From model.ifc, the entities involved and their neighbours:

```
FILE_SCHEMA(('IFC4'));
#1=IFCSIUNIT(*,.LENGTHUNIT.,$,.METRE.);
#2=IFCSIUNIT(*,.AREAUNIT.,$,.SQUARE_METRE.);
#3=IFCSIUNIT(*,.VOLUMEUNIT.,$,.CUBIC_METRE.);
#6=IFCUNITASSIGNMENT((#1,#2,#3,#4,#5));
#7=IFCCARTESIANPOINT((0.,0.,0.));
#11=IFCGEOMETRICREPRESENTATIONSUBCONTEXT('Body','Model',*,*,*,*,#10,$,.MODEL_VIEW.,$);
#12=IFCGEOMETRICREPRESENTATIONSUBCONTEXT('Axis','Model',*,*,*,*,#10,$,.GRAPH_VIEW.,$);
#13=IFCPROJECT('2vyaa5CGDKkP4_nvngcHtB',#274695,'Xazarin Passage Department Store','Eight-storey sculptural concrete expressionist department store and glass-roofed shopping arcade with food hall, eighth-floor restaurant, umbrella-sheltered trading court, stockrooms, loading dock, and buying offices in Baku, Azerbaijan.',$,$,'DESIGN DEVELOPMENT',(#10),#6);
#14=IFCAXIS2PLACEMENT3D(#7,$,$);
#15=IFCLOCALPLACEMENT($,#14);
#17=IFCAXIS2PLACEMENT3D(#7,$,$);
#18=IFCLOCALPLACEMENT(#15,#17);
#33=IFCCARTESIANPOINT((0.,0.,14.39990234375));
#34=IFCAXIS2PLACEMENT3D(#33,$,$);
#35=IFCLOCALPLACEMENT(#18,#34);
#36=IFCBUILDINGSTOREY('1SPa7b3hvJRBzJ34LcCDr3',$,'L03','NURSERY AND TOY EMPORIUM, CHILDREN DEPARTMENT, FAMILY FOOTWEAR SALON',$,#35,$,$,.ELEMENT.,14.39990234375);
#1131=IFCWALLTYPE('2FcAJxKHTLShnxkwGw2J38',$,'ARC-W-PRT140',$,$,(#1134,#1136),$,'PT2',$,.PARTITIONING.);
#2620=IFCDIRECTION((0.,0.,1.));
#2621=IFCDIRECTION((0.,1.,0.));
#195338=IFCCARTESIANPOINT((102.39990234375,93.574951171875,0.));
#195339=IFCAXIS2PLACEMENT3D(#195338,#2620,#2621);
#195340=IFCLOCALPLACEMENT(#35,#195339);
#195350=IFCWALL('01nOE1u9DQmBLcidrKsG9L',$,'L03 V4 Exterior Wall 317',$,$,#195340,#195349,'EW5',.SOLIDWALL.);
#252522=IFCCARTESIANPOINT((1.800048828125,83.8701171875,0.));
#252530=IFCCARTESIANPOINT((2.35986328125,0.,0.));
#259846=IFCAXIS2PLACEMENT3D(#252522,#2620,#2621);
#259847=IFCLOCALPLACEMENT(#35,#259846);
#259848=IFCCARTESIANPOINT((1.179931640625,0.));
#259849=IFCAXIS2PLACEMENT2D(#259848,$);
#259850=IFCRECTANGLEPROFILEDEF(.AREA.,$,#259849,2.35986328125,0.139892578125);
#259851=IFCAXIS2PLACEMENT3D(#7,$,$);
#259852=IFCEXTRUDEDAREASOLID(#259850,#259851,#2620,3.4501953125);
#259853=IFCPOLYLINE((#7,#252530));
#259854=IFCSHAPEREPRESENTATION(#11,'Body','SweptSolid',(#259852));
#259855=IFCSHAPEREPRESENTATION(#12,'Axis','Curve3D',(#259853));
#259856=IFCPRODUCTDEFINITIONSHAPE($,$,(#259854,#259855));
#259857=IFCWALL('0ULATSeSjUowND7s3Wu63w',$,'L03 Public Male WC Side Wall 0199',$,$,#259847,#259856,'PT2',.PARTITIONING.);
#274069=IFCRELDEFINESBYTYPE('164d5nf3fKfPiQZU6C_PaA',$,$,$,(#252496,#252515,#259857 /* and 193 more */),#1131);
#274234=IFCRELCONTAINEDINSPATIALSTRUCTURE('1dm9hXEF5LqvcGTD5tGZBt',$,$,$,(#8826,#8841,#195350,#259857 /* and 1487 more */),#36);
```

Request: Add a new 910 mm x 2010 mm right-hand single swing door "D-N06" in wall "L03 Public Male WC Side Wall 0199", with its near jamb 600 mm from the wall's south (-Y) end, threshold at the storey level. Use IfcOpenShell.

```python
import numpy as np
import ifcopenshell
import ifcopenshell.api.feature
import ifcopenshell.api.geometry
import ifcopenshell.api.root
import ifcopenshell.api.spatial
import ifcopenshell.geom
import ifcopenshell.util.element
import ifcopenshell.util.placement
import ifcopenshell.util.representation
import ifcopenshell.util.shape
import ifcopenshell.util.unit

model = ifcopenshell.open("model.ifc")
unit_scale = ifcopenshell.util.unit.calculate_unit_scale(model)
settings = ifcopenshell.geom.settings()


def volume(element):
    """Net volume in cubic metres, openings subtracted."""
    shape = ifcopenshell.geom.create_shape(settings, element)
    return ifcopenshell.util.shape.get_volume(shape.geometry)


wall = model.by_guid("0ULATSeSjUowND7s3Wu63w")
storey = ifcopenshell.util.element.get_container(wall, ifc_class="IfcBuildingStorey")
context = ifcopenshell.util.representation.get_context(model, "Model", "Body", "MODEL_VIEW")
before = volume(wall)

width, height, from_end, sill = 0.91, 2.01, 0.6, 0.0  # metres

# The wall runs along its own X axis, and the end named is its -X end.
wall_shape = ifcopenshell.geom.create_shape(settings, wall)
x, y, z = ifcopenshell.util.shape.get_vertices(wall_shape.geometry).T
start = x.min() + from_end
face, thickness = float(y.min()), float(y.max() - y.min())
wall_matrix = ifcopenshell.util.placement.get_local_placement(wall.ObjectPlacement)
level = ifcopenshell.util.placement.get_local_placement(storey.ObjectPlacement)[2, 3]


def in_wall(x, y):
    """Placement at x, y metres in the wall's axes, at sill height."""
    matrix = wall_matrix.copy()
    matrix[:, 3] = wall_matrix @ np.array([x / unit_scale, y / unit_scale, 0.0, 1.0])
    matrix[2, 3] = level + sill / unit_scale
    return matrix


# Opening: a box that overshoots both wall faces by 50 mm.
opening = ifcopenshell.api.root.create_entity(model, ifc_class="IfcOpeningElement", predefined_type="OPENING")
box = ifcopenshell.api.geometry.add_wall_representation(
    model, context=context, length=width, height=height, thickness=thickness + 0.1
)
ifcopenshell.api.geometry.assign_representation(model, product=opening, representation=box)
ifcopenshell.api.geometry.edit_object_placement(model, product=opening, matrix=in_wall(start, face - 0.05), is_si=False)
ifcopenshell.api.feature.add_feature(model, feature=opening, element=wall)

door = ifcopenshell.api.root.create_entity(model, ifc_class="IfcDoor", name="D-N06", predefined_type="DOOR")
door.OverallWidth, door.OverallHeight = width / unit_scale, height / unit_scale
door.OperationType = "SINGLE_SWING_RIGHT"
body = ifcopenshell.api.geometry.add_door_representation(
    model,
    context=context,
    overall_width=door.OverallWidth,
    overall_height=door.OverallHeight,
    operation_type="SINGLE_SWING_RIGHT",
    lining_properties={"LiningDepth": thickness / unit_scale, "ThresholdDepth": thickness / unit_scale},
)
ifcopenshell.api.geometry.assign_representation(model, product=door, representation=body)
ifcopenshell.api.spatial.assign_container(model, products=[door], relating_structure=storey)
ifcopenshell.api.feature.add_filling(model, opening=opening, element=door)

# The lining spans the wall, so the door starts at the wall face.
ifcopenshell.api.geometry.edit_object_placement(model, product=door, matrix=in_wall(start, face), is_si=False)

after = volume(wall)

print(f"wall volume {before:.3f} -> {after:.3f} m3")

model.write("model_rev.ifc")
```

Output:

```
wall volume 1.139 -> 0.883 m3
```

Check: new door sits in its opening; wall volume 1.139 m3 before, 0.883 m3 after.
